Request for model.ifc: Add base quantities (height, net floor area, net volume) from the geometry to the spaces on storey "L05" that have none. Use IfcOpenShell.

First a look at what the model holds.

```python
import ifcopenshell
import ifcopenshell.util.element
import ifcopenshell.util.unit

model = ifcopenshell.open("model.ifc")
print(model.schema)
for unit_type in ("LENGTHUNIT", "AREAUNIT", "VOLUMEUNIT"):
    print(unit_type, ifcopenshell.util.unit.calculate_unit_scale(model, unit_type))
storey = next(s for s in model.by_type("IfcBuildingStorey") if s.Name == "L05")
spaces = [e for e in ifcopenshell.util.element.get_decomposition(storey) if e.is_a("IfcSpace")]
for e in sorted(spaces, key=lambda e: e.id()):
    print(e.id(), e.is_a(), e.Name, list(ifcopenshell.util.element.get_psets(e, qtos_only=True)), sep=" | ")
```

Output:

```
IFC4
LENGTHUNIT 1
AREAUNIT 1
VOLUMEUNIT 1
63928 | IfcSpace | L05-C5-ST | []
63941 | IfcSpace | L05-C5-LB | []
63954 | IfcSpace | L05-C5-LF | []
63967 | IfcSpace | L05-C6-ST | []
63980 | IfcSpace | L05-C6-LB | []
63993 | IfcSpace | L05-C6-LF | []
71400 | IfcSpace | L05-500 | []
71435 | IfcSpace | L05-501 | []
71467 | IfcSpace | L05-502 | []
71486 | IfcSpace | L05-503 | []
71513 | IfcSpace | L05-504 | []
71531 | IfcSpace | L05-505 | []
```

```python
import ifcopenshell
import ifcopenshell.api.pset
import ifcopenshell.geom
import ifcopenshell.util.element
import ifcopenshell.util.shape
import ifcopenshell.util.unit

model = ifcopenshell.open("model.ifc")
unit_scale = ifcopenshell.util.unit.calculate_unit_scale(model)
area_scale = ifcopenshell.util.unit.calculate_unit_scale(model, "AREAUNIT")
volume_scale = ifcopenshell.util.unit.calculate_unit_scale(model, "VOLUMEUNIT")
settings = ifcopenshell.geom.settings()

storey = next(s for s in model.by_type("IfcBuildingStorey") if s.Name == "L05")
spaces = [e for e in ifcopenshell.util.element.get_decomposition(storey) if e.is_a("IfcSpace")]

for e in sorted(spaces, key=lambda e: e.id()):
    if ifcopenshell.util.element.get_psets(e, qtos_only=True, should_inherit=False):
        continue
    # Geometry comes back in metres, in the element's own axes.
    shape = ifcopenshell.geom.create_shape(settings, e)
    values = {
        "Height": ifcopenshell.util.shape.get_z(shape.geometry) / unit_scale,
        "NetFloorArea": ifcopenshell.util.shape.get_footprint_area(shape.geometry) / area_scale,
        "NetVolume": ifcopenshell.util.shape.get_volume(shape.geometry) / volume_scale,
    }
    qto = ifcopenshell.api.pset.add_qto(model, product=e, name="Qto_SpaceBaseQuantities")
    ifcopenshell.api.pset.edit_qto(model, qto=qto, properties=values)
    print(e.id(), {k: round(v, 3) for k, v in values.items()})

model.write("model_rev.ifc")
```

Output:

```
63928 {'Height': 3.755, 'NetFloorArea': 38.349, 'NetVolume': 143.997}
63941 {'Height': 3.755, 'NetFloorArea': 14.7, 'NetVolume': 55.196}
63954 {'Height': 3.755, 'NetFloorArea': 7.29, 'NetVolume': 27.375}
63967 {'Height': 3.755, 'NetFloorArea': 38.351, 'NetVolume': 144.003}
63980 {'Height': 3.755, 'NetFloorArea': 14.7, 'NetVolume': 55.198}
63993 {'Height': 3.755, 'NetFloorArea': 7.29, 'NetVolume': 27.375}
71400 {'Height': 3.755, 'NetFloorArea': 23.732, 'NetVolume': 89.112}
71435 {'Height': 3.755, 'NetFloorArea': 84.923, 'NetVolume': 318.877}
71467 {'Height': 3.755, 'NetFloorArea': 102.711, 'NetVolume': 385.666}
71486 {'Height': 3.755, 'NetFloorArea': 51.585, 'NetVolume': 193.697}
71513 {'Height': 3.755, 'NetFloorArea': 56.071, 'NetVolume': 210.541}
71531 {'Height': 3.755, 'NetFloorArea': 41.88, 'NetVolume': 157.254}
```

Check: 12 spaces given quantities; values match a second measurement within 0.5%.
